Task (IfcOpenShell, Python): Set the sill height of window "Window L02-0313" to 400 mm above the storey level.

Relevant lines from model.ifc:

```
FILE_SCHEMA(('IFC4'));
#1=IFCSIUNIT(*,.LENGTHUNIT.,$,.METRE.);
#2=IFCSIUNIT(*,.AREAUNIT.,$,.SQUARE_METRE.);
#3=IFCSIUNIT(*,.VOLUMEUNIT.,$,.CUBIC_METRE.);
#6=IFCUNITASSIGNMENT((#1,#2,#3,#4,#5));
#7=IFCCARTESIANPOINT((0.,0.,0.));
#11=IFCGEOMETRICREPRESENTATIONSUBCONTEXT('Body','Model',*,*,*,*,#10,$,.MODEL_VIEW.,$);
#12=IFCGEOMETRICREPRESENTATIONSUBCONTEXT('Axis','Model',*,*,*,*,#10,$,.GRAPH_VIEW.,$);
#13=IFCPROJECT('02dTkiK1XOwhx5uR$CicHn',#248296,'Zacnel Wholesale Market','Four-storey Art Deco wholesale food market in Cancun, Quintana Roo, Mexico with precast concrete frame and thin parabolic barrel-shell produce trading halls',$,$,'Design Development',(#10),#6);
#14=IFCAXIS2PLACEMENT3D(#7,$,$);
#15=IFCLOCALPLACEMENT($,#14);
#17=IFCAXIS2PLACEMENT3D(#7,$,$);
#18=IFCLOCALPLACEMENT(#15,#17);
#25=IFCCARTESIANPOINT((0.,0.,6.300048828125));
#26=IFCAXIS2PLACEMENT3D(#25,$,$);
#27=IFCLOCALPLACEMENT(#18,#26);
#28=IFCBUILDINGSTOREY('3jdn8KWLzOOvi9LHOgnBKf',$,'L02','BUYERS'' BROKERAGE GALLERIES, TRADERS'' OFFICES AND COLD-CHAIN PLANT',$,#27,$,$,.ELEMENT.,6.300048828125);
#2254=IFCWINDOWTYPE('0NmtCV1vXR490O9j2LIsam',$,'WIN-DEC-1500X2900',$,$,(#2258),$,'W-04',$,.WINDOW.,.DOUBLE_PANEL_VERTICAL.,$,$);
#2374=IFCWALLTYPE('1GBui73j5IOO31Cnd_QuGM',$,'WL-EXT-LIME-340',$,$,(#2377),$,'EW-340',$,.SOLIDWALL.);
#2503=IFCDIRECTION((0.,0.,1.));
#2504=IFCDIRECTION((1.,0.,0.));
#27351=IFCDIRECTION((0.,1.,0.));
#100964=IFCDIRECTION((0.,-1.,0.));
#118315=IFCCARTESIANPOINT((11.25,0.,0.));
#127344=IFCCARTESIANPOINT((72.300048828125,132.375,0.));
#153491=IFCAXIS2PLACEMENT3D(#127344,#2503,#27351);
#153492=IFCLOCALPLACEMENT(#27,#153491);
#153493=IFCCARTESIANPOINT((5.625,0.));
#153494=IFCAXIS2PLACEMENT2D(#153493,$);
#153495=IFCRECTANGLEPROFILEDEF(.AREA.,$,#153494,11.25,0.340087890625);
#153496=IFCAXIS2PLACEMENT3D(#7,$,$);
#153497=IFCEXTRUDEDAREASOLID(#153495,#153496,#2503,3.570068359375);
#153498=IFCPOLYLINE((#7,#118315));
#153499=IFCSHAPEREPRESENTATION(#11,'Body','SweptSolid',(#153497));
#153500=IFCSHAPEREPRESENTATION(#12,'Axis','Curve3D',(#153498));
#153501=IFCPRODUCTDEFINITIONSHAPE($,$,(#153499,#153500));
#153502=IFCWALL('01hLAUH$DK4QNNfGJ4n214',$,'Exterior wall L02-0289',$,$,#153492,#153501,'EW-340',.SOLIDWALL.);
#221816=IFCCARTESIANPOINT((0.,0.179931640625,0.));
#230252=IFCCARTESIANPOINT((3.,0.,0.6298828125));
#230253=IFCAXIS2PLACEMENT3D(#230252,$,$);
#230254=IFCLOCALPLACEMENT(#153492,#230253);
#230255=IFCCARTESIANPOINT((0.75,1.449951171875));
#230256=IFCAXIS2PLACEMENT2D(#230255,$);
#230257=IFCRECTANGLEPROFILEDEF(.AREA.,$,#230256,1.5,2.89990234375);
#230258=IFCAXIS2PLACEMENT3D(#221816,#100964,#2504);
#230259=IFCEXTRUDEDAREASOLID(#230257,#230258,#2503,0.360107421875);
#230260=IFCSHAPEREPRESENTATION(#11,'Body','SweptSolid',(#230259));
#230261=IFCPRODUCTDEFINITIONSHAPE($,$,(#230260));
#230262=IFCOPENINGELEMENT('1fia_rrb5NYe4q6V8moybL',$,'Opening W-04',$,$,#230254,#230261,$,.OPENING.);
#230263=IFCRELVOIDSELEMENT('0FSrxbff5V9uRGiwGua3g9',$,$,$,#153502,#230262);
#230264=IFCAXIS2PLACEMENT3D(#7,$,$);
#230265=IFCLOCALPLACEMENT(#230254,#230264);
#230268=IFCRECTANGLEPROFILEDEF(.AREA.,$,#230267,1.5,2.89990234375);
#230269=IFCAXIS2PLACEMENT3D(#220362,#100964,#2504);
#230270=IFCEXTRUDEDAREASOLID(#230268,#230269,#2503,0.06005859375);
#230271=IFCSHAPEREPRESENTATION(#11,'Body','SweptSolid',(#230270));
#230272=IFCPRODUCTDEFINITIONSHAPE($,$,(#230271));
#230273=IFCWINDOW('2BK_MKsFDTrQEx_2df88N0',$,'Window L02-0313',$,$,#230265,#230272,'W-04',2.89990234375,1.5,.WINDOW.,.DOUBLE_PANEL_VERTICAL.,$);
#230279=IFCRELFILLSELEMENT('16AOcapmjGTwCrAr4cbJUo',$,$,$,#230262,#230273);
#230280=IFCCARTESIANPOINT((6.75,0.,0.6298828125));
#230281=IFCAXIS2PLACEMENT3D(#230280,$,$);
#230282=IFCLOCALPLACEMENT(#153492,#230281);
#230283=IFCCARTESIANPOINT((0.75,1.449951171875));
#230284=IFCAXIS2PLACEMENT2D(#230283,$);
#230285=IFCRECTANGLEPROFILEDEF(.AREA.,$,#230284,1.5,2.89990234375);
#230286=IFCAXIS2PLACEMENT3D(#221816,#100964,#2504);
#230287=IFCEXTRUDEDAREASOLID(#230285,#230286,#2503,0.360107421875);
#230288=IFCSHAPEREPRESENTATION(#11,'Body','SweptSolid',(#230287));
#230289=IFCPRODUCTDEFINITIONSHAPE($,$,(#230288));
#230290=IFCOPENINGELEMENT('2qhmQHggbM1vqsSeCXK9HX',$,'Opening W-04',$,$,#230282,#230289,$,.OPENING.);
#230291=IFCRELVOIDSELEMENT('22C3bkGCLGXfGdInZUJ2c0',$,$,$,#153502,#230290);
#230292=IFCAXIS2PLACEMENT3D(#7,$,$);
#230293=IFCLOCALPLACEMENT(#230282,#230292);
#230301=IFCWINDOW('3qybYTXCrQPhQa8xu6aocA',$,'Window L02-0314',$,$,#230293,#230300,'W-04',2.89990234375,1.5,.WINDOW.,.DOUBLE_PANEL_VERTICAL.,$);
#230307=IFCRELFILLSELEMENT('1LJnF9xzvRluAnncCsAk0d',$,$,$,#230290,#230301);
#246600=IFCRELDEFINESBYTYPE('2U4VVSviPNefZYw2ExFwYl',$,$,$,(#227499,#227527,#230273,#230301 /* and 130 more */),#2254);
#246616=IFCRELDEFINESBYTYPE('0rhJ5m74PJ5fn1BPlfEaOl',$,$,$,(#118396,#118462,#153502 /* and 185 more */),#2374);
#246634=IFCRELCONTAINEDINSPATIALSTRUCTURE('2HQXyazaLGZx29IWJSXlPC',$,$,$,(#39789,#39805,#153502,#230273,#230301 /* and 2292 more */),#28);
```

```python
import numpy as np
import ifcopenshell
import ifcopenshell.api.geometry
import ifcopenshell.geom
import ifcopenshell.util.element
import ifcopenshell.util.placement
import ifcopenshell.util.shape
import ifcopenshell.util.unit

model = ifcopenshell.open("model.ifc")
unit_scale = ifcopenshell.util.unit.calculate_unit_scale(model)

window = model.by_id(230273)
opening = window.FillsVoids[0].RelatingOpeningElement
storey = ifcopenshell.util.element.get_container(window, ifc_class="IfcBuildingStorey")
level = ifcopenshell.util.placement.get_local_placement(storey.ObjectPlacement)[2, 3]

# The opening's origin need not be at the sill, so measure its lowest point.
shape = ifcopenshell.geom.create_shape(ifcopenshell.geom.settings(), opening)
bottom = ifcopenshell.util.shape.get_shape_bottom_elevation(shape, shape.geometry) / unit_scale
dz = level + 0.4 / unit_scale - bottom

shift = np.array([0.0, 0.0, dz])
# The window is placed relative to its opening, so it follows when the opening moves.
matrix = ifcopenshell.util.placement.get_local_placement(opening.ObjectPlacement)
matrix[:3, 3] += shift
ifcopenshell.api.geometry.edit_object_placement(
    model, product=opening, matrix=matrix, is_si=False, should_transform_children=True
)

print(f"moved by {dz * unit_scale:+.3f} m")

model.write("model_edited.ifc")
```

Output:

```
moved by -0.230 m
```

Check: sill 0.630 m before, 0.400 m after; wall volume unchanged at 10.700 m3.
